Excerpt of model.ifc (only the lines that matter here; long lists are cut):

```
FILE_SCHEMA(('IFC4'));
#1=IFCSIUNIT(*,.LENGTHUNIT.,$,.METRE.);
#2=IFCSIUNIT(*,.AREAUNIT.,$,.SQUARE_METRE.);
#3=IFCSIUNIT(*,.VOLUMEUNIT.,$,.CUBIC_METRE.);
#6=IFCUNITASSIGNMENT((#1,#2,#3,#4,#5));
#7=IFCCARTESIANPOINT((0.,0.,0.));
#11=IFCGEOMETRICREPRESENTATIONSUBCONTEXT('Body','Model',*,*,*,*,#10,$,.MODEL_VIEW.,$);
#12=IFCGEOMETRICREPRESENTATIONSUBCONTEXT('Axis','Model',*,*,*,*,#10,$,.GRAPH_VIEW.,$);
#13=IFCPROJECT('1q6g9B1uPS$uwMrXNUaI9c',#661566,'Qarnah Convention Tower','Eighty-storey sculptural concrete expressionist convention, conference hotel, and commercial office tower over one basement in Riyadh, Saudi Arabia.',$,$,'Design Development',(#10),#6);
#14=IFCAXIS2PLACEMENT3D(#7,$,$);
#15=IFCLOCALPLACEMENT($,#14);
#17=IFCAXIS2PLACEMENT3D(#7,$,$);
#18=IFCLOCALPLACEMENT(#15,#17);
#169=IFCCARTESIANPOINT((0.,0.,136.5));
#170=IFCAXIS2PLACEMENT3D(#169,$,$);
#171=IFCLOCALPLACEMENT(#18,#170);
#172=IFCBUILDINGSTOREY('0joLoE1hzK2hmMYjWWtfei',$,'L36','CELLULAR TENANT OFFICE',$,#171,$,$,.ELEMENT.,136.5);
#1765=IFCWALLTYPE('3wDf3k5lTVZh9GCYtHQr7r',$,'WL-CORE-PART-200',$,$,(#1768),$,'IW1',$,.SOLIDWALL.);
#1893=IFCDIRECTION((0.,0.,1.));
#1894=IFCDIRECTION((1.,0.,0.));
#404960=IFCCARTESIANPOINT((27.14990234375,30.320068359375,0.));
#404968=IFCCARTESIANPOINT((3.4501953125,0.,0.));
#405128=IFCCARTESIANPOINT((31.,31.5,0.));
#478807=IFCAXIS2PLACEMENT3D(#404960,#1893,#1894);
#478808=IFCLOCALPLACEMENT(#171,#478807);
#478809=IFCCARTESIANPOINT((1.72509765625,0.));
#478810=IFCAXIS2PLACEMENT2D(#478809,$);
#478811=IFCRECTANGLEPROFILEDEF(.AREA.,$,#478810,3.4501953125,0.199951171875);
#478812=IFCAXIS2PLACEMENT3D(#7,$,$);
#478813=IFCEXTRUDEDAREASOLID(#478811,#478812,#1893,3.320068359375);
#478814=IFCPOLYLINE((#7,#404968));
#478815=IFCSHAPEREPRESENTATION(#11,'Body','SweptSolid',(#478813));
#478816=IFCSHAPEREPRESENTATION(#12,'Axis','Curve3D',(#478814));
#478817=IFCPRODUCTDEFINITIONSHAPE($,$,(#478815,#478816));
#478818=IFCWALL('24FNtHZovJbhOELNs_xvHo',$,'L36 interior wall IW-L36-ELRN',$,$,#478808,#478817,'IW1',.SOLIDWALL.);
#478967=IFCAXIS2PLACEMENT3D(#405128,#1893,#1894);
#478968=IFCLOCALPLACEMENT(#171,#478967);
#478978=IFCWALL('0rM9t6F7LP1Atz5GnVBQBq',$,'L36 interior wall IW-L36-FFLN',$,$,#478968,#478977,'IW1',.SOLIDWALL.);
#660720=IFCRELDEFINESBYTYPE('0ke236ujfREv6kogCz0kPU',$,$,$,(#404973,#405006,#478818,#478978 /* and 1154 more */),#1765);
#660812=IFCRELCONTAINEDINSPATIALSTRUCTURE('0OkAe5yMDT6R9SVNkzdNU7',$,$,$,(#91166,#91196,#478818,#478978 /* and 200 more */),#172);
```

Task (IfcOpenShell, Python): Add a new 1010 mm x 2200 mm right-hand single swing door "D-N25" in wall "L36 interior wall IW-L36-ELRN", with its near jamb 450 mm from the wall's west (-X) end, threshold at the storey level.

```python
import numpy as np
import ifcopenshell
import ifcopenshell.api.feature
import ifcopenshell.api.geometry
import ifcopenshell.api.root
import ifcopenshell.api.spatial
import ifcopenshell.geom
import ifcopenshell.util.element
import ifcopenshell.util.placement
import ifcopenshell.util.representation
import ifcopenshell.util.shape
import ifcopenshell.util.unit

model = ifcopenshell.open("model.ifc")
unit_scale = ifcopenshell.util.unit.calculate_unit_scale(model)
settings = ifcopenshell.geom.settings()


def volume(element):
    """Net volume in cubic metres, openings subtracted."""
    shape = ifcopenshell.geom.create_shape(settings, element)
    return ifcopenshell.util.shape.get_volume(shape.geometry)


wall = model.by_id(478818)
storey = ifcopenshell.util.element.get_container(wall, ifc_class="IfcBuildingStorey")
context = ifcopenshell.util.representation.get_context(model, "Model", "Body", "MODEL_VIEW")
before = volume(wall)

width, height, from_end, sill = 1.01, 2.2, 0.45, 0.0  # metres

# The wall runs along its own X axis, and the end named is its -X end.
wall_shape = ifcopenshell.geom.create_shape(settings, wall)
x, y, z = ifcopenshell.util.shape.get_vertices(wall_shape.geometry).T
start = x.min() + from_end
face, thickness = float(y.min()), float(y.max() - y.min())
wall_matrix = ifcopenshell.util.placement.get_local_placement(wall.ObjectPlacement)
level = ifcopenshell.util.placement.get_local_placement(storey.ObjectPlacement)[2, 3]


def in_wall(x, y):
    """Placement at x, y metres in the wall's axes, at sill height."""
    matrix = wall_matrix.copy()
    matrix[:, 3] = wall_matrix @ np.array([x / unit_scale, y / unit_scale, 0.0, 1.0])
    matrix[2, 3] = level + sill / unit_scale
    return matrix


# Opening: a box that overshoots both wall faces by 50 mm.
opening = ifcopenshell.api.root.create_entity(model, ifc_class="IfcOpeningElement", predefined_type="OPENING")
box = ifcopenshell.api.geometry.add_wall_representation(
    model, context=context, length=width, height=height, thickness=thickness + 0.1
)
ifcopenshell.api.geometry.assign_representation(model, product=opening, representation=box)
ifcopenshell.api.geometry.edit_object_placement(model, product=opening, matrix=in_wall(start, face - 0.05), is_si=False)
ifcopenshell.api.feature.add_feature(model, feature=opening, element=wall)

door = ifcopenshell.api.root.create_entity(model, ifc_class="IfcDoor", name="D-N25", predefined_type="DOOR")
door.OverallWidth, door.OverallHeight = width / unit_scale, height / unit_scale
door.OperationType = "SINGLE_SWING_RIGHT"
body = ifcopenshell.api.geometry.add_door_representation(
    model,
    context=context,
    overall_width=door.OverallWidth,
    overall_height=door.OverallHeight,
    operation_type="SINGLE_SWING_RIGHT",
    lining_properties={"LiningDepth": thickness / unit_scale, "ThresholdDepth": thickness / unit_scale},
)
ifcopenshell.api.geometry.assign_representation(model, product=door, representation=body)
ifcopenshell.api.spatial.assign_container(model, products=[door], relating_structure=storey)
ifcopenshell.api.feature.add_filling(model, opening=opening, element=door)

# The lining spans the wall, so the door starts at the wall face.
ifcopenshell.api.geometry.edit_object_placement(model, product=door, matrix=in_wall(start, face), is_si=False)

after = volume(wall)

print(f"wall volume {before:.3f} -> {after:.3f} m3")

model.write("model_rev.ifc")
```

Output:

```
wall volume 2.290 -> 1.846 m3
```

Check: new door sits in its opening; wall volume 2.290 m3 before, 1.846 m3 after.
